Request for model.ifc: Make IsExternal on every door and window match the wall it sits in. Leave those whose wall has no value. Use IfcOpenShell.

First a look at what the model holds.

```python
import ifcopenshell
import ifcopenshell.util.element

model = ifcopenshell.open("model.ifc")
print(model.schema)
seen = {}
for e in model.by_type("IfcDoor") + model.by_type("IfcWindow"):
    if not e.FillsVoids:
        continue
    host = e.FillsVoids[0].RelatingOpeningElement.VoidsElements[0].RelatingBuildingElement
    own = ifcopenshell.util.element.get_pset(e, f"Pset_{e.is_a()[3:].removesuffix('StandardCase')}Common", "IsExternal")
    wall = ifcopenshell.util.element.get_pset(host, "Pset_WallCommon", "IsExternal")
    seen[e.is_a(), own, wall] = seen.get((e.is_a(), own, wall), 0) + 1
for (cls, own, wall), count in sorted(seen.items(), key=str):
    print(count, cls, "IsExternal:", own, "| host wall:", wall)
```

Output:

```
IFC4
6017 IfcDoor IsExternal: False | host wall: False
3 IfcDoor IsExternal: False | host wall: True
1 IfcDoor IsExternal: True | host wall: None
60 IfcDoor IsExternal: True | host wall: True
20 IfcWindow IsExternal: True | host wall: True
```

```python
import ifcopenshell
import ifcopenshell.api.pset
import ifcopenshell.util.element

model = ifcopenshell.open("model.ifc")

count = 0
for ifc_class, pset_name in (("IfcDoor", "Pset_DoorCommon"), ("IfcWindow", "Pset_WindowCommon")):
    for e in model.by_type(ifc_class):
        if not e.FillsVoids:
            continue
        host = e.FillsVoids[0].RelatingOpeningElement.VoidsElements[0].RelatingBuildingElement
        external = ifcopenshell.util.element.get_pset(host, "Pset_WallCommon", "IsExternal")
        if external is None or ifcopenshell.util.element.get_pset(e, pset_name, "IsExternal") == external:
            continue
        pset = ifcopenshell.api.pset.add_pset(model, product=e, name=pset_name)
        ifcopenshell.api.pset.edit_pset(model, pset=pset, properties={"IsExternal": external})
        count += 1

print(count, "updated")

model.write("model_v2.ifc")
```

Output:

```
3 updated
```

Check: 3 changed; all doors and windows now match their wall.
